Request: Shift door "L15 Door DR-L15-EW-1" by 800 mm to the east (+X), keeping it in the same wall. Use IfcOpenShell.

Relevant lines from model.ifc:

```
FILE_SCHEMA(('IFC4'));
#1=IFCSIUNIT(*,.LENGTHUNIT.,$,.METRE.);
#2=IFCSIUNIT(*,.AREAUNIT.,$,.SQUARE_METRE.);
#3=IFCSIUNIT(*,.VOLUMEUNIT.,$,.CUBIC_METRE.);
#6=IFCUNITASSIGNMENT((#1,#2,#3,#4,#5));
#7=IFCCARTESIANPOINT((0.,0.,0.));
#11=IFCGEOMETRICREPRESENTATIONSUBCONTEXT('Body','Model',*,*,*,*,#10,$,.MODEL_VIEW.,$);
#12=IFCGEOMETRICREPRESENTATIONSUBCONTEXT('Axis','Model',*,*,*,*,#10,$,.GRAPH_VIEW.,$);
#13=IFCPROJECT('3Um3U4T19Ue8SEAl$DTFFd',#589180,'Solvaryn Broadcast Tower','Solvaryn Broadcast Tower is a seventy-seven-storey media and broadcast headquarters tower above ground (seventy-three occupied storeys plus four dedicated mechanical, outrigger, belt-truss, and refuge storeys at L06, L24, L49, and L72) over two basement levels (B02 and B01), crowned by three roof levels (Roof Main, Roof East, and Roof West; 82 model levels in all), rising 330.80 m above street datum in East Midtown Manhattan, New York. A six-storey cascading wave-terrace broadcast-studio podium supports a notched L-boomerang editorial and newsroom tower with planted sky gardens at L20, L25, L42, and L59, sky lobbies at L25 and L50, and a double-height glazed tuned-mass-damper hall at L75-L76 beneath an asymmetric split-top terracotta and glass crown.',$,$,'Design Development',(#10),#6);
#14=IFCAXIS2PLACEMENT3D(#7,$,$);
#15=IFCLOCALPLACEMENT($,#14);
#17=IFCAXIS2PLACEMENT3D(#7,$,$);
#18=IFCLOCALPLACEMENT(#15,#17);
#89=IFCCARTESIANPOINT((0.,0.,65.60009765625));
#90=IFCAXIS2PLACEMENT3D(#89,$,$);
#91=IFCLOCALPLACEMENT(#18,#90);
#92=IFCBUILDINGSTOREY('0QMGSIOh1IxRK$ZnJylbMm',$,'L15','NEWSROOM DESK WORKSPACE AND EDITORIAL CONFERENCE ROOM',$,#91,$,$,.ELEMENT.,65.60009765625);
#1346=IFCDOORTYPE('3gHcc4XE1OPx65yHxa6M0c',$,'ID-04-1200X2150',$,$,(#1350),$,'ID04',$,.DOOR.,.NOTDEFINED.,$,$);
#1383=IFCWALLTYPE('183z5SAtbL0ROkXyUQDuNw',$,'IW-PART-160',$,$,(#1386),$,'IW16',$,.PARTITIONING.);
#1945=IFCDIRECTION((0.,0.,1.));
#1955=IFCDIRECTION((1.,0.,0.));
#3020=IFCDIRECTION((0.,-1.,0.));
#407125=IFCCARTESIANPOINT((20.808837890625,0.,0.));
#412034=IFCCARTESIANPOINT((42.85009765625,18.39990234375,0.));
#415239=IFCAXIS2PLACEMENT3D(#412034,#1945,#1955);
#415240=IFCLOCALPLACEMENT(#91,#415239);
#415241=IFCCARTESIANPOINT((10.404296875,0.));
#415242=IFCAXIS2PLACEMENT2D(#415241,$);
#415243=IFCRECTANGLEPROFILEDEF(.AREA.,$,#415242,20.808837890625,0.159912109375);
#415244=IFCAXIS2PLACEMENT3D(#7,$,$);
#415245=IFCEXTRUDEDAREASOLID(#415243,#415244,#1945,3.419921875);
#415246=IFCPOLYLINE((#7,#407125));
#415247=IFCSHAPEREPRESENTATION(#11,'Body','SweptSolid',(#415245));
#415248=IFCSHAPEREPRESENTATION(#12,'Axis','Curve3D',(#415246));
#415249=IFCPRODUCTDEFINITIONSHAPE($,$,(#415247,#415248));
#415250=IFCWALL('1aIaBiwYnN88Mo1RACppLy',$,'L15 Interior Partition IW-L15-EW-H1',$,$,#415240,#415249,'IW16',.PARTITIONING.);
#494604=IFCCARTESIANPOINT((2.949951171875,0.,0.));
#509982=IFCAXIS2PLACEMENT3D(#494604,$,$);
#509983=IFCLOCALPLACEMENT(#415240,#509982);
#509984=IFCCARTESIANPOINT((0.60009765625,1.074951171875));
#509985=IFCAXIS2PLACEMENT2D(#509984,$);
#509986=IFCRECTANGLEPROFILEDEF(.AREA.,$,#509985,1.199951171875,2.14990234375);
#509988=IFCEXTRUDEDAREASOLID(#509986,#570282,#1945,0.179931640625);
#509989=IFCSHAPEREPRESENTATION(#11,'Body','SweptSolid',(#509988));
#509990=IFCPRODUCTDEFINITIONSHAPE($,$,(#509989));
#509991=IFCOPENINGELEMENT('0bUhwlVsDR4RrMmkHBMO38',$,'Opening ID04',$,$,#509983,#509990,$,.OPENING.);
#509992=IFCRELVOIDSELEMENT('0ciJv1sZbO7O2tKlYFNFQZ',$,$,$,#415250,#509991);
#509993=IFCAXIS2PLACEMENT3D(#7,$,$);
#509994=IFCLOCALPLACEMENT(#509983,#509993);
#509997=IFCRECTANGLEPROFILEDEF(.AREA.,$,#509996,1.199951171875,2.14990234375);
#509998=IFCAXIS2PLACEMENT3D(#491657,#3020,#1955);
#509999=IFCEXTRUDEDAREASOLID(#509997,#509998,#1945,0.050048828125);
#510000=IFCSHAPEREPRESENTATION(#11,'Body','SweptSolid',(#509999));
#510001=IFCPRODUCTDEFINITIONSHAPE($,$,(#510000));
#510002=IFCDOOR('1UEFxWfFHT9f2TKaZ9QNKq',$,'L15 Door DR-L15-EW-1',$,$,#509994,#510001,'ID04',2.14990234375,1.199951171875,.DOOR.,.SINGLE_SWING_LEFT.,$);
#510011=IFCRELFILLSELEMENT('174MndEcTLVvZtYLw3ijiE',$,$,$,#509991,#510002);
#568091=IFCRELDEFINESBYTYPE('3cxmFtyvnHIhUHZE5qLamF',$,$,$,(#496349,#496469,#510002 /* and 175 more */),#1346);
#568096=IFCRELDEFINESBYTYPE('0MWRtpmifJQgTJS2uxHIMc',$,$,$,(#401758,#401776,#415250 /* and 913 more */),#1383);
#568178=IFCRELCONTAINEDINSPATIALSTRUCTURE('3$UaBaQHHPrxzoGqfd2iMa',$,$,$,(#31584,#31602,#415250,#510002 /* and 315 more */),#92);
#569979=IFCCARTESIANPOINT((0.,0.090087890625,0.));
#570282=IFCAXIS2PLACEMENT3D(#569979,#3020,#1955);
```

```python
import ifcopenshell
import ifcopenshell.api.geometry
import ifcopenshell.util.placement
import ifcopenshell.util.unit

model = ifcopenshell.open("model.ifc")
unit_scale = ifcopenshell.util.unit.calculate_unit_scale(model)

door = model.by_id(510002)
opening = door.FillsVoids[0].RelatingOpeningElement
wall = opening.VoidsElements[0].RelatingBuildingElement

wall_matrix = ifcopenshell.util.placement.get_local_placement(wall.ObjectPlacement)
shift = wall_matrix[:3, 0] * 0.8 / unit_scale
before = ifcopenshell.util.placement.get_local_placement(door.ObjectPlacement)[:3, 3].copy()

# The door is placed relative to its opening, so it follows when the opening moves.
matrix = ifcopenshell.util.placement.get_local_placement(opening.ObjectPlacement)
matrix[:3, 3] += shift
ifcopenshell.api.geometry.edit_object_placement(
    model, product=opening, matrix=matrix, is_si=False, should_transform_children=True
)

after = ifcopenshell.util.placement.get_local_placement(door.ObjectPlacement)[:3, 3]
print("door moved by", (after - before).round(3) + 0.0)

model.write("model-out.ifc")
```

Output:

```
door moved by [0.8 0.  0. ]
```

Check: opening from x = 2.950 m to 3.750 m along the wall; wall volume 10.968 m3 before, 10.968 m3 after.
